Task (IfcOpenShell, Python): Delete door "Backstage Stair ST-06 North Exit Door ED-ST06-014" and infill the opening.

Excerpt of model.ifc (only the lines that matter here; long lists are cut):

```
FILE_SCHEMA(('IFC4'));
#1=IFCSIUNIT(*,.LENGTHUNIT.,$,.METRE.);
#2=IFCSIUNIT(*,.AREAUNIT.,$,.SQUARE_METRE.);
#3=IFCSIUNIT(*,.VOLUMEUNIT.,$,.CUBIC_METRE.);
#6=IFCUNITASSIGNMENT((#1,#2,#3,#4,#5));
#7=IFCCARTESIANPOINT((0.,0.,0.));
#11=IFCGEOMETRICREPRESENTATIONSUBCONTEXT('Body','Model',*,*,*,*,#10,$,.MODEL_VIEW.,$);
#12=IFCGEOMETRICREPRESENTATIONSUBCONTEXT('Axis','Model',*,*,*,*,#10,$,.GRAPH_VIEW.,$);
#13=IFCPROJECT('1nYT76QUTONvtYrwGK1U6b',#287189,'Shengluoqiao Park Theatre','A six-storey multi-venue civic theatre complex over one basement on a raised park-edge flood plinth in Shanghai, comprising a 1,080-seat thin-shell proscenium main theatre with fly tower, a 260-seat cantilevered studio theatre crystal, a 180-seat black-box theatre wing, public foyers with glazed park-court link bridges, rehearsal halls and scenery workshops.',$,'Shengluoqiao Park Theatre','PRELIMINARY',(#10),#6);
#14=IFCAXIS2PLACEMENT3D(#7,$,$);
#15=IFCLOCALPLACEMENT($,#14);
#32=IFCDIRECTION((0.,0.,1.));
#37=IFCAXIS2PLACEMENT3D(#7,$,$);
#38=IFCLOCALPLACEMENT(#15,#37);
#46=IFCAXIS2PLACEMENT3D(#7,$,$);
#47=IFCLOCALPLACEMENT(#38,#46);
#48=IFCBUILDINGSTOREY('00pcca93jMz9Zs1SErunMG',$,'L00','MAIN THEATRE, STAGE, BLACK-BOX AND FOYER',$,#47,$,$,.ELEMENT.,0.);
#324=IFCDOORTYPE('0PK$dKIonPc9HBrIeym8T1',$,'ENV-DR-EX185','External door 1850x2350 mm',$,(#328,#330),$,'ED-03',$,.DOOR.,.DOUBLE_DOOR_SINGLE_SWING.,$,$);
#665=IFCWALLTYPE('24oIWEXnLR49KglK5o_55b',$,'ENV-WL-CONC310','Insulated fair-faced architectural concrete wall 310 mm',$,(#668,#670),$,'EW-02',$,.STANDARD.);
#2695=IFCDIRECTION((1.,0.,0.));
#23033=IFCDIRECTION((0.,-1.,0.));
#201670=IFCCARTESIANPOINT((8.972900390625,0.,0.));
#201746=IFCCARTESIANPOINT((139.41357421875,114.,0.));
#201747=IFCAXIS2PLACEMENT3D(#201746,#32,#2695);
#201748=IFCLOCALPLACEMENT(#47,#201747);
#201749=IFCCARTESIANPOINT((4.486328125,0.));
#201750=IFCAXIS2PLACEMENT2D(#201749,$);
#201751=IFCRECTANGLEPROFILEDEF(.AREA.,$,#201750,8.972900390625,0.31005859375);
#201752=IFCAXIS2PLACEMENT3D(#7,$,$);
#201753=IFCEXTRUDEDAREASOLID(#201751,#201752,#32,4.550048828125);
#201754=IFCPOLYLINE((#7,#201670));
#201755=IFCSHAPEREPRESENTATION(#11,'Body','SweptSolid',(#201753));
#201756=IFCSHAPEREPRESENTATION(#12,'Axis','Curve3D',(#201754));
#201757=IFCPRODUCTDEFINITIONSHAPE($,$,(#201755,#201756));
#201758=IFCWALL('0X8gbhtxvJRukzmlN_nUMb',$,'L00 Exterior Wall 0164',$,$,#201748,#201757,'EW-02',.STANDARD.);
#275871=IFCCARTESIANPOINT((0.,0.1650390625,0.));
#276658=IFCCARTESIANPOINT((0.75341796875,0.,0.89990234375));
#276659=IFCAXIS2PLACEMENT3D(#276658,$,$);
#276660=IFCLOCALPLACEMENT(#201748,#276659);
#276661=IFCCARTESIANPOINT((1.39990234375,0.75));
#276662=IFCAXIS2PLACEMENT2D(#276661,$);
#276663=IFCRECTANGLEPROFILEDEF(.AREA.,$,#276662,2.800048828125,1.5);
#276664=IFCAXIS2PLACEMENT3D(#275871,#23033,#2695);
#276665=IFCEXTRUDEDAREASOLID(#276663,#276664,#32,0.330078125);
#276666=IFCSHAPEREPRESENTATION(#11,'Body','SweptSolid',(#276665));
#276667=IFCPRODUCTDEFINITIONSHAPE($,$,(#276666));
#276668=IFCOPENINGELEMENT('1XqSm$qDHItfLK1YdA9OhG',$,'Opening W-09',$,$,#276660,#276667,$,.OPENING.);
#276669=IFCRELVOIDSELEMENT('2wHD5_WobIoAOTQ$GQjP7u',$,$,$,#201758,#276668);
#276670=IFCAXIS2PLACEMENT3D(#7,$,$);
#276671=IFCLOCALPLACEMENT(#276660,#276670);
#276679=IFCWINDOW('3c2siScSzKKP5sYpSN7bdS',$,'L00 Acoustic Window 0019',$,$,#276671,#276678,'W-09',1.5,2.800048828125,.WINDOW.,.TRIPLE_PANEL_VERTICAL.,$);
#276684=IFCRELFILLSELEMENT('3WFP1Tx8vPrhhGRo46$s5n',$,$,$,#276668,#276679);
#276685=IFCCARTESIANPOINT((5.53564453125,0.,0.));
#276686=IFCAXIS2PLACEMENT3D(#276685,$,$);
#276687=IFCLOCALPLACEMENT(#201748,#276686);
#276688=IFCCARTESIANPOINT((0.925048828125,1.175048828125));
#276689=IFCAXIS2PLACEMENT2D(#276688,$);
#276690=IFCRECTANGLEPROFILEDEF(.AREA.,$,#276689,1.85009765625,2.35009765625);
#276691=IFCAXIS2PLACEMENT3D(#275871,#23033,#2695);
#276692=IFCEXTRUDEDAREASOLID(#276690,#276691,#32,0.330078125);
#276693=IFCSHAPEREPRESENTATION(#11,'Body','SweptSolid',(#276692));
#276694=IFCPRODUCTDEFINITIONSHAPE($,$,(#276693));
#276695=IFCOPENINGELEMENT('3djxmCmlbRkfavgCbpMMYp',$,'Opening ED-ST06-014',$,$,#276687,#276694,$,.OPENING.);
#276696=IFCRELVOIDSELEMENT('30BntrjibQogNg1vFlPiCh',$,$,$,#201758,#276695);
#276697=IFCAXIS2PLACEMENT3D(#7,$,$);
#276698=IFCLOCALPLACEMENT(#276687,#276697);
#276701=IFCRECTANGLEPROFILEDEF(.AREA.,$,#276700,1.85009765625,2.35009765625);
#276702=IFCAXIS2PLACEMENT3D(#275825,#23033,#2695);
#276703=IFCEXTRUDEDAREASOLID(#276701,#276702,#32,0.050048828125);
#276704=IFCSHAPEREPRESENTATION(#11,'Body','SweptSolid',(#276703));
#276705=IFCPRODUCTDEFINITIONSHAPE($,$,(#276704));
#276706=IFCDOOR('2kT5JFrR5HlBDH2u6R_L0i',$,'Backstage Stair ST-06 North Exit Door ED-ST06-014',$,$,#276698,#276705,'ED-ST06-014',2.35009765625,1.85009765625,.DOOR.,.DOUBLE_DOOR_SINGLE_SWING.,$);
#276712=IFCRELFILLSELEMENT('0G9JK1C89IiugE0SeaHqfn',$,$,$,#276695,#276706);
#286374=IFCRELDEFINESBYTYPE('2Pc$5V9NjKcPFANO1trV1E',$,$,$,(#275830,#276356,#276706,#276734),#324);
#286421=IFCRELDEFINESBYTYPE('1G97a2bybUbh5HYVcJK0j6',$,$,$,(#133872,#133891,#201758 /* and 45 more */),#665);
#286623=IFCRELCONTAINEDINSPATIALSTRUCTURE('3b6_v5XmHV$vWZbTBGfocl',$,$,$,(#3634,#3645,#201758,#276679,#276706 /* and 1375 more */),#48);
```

```python
import ifcopenshell
import ifcopenshell.api.feature
import ifcopenshell.api.root
import ifcopenshell.geom
import ifcopenshell.util.shape

model = ifcopenshell.open("model.ifc")
settings = ifcopenshell.geom.settings()


def volume(element):
    """Net volume in cubic metres, openings subtracted."""
    shape = ifcopenshell.geom.create_shape(settings, element)
    return ifcopenshell.util.shape.get_volume(shape.geometry)


door = model.by_guid("2kT5JFrR5HlBDH2u6R_L0i")
opening = door.FillsVoids[0].RelatingOpeningElement
wall = opening.VoidsElements[0].RelatingBuildingElement
before = volume(wall)

ifcopenshell.api.root.remove_product(model, product=door)
ifcopenshell.api.feature.remove_feature(model, feature=opening)

after = volume(wall)

print(f"wall volume {before:.3f} -> {after:.3f} m3")

model.write("model-out.ifc")
```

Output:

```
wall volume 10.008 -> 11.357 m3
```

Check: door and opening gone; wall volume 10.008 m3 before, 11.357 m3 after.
